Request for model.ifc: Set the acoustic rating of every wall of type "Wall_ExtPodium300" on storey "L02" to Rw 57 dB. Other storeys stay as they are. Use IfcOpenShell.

First a look at what the model holds.

```python
import ifcopenshell
import ifcopenshell.util.element

model = ifcopenshell.open("model.ifc")
print(model.schema)
storey = next(s for s in model.by_type("IfcBuildingStorey") if s.Name == "L02")
walls = [e for e in ifcopenshell.util.element.get_decomposition(storey) if e.is_a("IfcWall")]
seen = {}
for e in walls:
    element_type = ifcopenshell.util.element.get_type(e)
    key = (element_type.Name if element_type != e and element_type else None, ifcopenshell.util.element.get_pset(e, "Pset_WallCommon", "AcousticRating"))
    seen[key] = seen.get(key, 0) + 1
for (name, value), count in sorted(seen.items(), key=str):
    print(count, "x", name, "|", value)
```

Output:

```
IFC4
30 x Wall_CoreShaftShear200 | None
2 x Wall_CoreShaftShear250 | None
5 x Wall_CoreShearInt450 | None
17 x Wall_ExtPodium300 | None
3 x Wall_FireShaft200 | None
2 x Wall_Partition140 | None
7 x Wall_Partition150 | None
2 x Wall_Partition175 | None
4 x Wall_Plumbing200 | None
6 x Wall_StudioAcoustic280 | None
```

```python
import ifcopenshell
import ifcopenshell.api.pset
import ifcopenshell.util.element

model = ifcopenshell.open("model.ifc")

storey = next(s for s in model.by_type("IfcBuildingStorey") if s.Name == "L02")
walls = [e for e in ifcopenshell.util.element.get_decomposition(storey) if e.is_a("IfcWall")]

count = 0
for e in walls:
    element_type = ifcopenshell.util.element.get_type(e)
    if element_type in (None, e) or element_type.Name != "Wall_ExtPodium300":
        continue
    found = ifcopenshell.util.element.get_pset(e, "Pset_WallCommon", should_inherit=False)
    if found:
        pset = model.by_id(found["id"])
        if len(ifcopenshell.util.element.get_elements_by_pset(pset)) > 1:
            pset = ifcopenshell.api.pset.unshare_pset(model, products=[e], pset=pset)[0]
    else:
        pset = ifcopenshell.api.pset.add_pset(model, product=e, name="Pset_WallCommon")
    ifcopenshell.api.pset.edit_pset(model, pset=pset, properties={"AcousticRating": "Rw 57 dB"})
    count += 1

print(count, "walls updated")

model.write("model-out.ifc")
```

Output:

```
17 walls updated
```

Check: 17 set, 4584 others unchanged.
